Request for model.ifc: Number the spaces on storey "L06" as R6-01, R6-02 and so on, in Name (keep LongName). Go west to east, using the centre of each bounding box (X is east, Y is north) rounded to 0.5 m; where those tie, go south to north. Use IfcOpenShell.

First a look at what the model holds.

```python
import ifcopenshell
import ifcopenshell.util.element
import ifcopenshell.util.placement

model = ifcopenshell.open("model.ifc")
print(model.schema)
storey = next(s for s in model.by_type("IfcBuildingStorey") if s.Name == "L06")
spaces = [e for e in ifcopenshell.util.element.get_decomposition(storey) if e.is_a("IfcSpace")]
for e in sorted(spaces, key=lambda e: e.id()):
    origin = ifcopenshell.util.placement.get_local_placement(e.ObjectPlacement)[:3, 3]
    print(e.id(), e.Name, e.LongName, origin.round(2) + 0.0, sep=" | ")
```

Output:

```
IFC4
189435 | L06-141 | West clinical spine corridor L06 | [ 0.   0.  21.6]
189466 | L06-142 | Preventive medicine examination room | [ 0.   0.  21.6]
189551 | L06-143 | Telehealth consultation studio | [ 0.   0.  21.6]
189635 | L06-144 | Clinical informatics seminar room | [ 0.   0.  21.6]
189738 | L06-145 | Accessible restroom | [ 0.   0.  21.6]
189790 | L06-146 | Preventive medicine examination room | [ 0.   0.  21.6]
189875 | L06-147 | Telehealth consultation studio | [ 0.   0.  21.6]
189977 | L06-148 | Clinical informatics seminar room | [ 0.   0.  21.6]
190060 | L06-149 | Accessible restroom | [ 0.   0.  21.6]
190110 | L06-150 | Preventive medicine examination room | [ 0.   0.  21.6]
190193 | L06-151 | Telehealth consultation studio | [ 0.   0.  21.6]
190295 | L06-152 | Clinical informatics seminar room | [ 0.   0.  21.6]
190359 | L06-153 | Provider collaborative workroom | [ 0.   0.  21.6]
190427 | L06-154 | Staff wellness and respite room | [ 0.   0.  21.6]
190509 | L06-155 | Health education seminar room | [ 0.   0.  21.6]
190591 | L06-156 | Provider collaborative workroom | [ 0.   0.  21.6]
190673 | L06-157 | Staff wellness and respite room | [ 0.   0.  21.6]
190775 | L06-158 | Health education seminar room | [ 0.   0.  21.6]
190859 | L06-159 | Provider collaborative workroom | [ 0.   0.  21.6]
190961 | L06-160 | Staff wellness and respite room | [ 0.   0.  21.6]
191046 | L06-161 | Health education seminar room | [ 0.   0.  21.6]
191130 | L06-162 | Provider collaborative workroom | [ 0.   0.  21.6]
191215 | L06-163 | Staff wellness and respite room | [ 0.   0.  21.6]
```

```python
import ifcopenshell
import ifcopenshell.geom
import ifcopenshell.util.element
import ifcopenshell.util.shape

model = ifcopenshell.open("model.ifc")
settings = ifcopenshell.geom.settings()
settings.set("use-world-coords", True)


def centre(element):
    shape = ifcopenshell.geom.create_shape(settings, element)
    return ifcopenshell.util.shape.get_bbox_centroid(shape.geometry)


storey = next(s for s in model.by_type("IfcBuildingStorey") if s.Name == "L06")
spaces = [e for e in ifcopenshell.util.element.get_decomposition(storey) if e.is_a("IfcSpace")]

# Insertion points can sit at a corner or the storey origin, so sort by the geometry (in metres).
centres = {e: centre(e) for e in spaces}
spaces.sort(key=lambda e: (round(centres[e][0] / 0.5), centres[e][1]))

for i, e in enumerate(spaces, start=1):
    number = f"R6-{i:02d}"
    e.Name = number
    print(e.id(), number)

model.write("model-out.ifc")
```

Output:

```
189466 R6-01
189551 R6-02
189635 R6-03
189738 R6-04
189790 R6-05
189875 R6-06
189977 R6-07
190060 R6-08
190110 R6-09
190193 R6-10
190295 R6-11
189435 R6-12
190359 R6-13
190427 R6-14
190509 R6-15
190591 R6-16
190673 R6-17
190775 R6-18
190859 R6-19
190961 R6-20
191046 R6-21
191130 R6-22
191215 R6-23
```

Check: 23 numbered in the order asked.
